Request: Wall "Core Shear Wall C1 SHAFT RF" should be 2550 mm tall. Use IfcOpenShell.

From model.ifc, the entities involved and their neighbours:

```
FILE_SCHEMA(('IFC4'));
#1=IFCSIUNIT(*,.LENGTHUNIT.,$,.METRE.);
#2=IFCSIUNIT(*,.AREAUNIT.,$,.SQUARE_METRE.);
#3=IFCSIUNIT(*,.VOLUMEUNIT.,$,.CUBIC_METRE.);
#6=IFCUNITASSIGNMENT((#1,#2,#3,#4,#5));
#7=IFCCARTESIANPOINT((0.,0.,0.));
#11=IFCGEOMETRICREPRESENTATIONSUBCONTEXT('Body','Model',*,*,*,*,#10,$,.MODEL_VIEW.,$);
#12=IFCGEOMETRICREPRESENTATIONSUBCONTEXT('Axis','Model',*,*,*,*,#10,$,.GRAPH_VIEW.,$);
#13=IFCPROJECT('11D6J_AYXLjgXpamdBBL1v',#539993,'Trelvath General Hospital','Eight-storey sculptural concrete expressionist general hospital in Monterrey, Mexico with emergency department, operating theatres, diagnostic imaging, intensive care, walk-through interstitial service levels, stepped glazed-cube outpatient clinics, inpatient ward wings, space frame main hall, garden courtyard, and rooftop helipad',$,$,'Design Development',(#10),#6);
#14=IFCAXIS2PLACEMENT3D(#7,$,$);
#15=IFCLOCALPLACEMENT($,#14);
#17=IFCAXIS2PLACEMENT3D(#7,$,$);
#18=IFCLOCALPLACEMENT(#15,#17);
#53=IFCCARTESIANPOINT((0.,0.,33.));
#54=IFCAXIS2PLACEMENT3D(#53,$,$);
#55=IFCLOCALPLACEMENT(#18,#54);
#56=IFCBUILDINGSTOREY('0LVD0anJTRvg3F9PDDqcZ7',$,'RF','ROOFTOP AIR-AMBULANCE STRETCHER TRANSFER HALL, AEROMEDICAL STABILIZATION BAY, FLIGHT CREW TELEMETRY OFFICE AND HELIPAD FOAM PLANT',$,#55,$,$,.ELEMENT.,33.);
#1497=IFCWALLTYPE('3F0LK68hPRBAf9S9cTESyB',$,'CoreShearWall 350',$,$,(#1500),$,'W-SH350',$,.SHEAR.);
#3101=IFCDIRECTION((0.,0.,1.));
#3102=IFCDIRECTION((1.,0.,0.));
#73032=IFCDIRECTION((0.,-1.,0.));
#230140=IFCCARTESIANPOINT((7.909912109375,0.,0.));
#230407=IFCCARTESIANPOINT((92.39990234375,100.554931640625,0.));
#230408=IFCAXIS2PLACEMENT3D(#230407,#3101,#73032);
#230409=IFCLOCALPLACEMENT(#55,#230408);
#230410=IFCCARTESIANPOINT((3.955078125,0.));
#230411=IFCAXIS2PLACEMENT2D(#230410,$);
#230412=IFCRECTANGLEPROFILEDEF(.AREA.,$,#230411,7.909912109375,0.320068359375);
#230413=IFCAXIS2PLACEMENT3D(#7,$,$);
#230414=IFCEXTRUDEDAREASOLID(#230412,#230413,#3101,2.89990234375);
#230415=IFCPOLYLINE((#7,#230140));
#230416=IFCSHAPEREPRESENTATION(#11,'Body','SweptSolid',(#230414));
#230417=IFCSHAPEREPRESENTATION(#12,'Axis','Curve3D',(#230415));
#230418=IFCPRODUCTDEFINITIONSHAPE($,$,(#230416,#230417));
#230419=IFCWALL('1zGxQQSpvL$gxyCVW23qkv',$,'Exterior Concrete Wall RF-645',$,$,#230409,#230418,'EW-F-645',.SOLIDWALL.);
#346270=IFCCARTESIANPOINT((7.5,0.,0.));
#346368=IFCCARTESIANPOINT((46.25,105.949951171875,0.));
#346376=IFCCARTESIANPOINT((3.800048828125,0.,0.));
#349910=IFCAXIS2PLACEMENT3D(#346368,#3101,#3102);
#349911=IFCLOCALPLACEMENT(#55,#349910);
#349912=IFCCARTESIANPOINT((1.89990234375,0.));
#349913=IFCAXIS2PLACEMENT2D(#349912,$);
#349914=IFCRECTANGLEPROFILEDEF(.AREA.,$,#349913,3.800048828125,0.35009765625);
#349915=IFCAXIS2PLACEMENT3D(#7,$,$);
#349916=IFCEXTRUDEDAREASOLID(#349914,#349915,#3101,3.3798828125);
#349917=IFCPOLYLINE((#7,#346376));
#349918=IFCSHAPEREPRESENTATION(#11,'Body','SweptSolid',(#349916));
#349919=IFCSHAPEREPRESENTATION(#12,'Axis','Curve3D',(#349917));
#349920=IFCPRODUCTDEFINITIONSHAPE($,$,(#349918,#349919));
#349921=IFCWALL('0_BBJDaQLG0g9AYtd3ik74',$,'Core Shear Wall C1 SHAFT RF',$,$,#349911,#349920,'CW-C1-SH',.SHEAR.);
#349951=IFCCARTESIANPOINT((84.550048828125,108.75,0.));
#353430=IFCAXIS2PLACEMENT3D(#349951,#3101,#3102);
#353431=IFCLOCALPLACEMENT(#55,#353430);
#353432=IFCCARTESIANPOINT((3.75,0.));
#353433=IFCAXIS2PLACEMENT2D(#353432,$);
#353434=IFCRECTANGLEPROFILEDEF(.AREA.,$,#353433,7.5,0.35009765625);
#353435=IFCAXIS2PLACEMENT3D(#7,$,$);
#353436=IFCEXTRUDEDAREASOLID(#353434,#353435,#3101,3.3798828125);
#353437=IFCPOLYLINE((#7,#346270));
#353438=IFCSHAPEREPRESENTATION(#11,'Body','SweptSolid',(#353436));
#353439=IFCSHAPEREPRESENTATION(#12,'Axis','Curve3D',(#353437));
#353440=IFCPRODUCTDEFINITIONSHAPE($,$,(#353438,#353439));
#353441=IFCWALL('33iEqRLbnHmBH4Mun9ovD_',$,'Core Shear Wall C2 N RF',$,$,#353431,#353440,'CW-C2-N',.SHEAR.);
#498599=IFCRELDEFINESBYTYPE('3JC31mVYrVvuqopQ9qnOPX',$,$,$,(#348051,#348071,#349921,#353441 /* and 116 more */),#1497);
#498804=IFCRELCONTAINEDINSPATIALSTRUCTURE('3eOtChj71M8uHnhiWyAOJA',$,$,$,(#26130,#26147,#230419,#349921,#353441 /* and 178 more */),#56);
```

```python
import ifcopenshell
import ifcopenshell.geom
import ifcopenshell.util.representation
import ifcopenshell.util.shape
import ifcopenshell.util.unit

model = ifcopenshell.open("model.ifc")
unit_scale = ifcopenshell.util.unit.calculate_unit_scale(model)
settings = ifcopenshell.geom.settings()


def volume(element):
    """Net volume in cubic metres, openings subtracted."""
    shape = ifcopenshell.geom.create_shape(settings, element)
    return ifcopenshell.util.shape.get_volume(shape.geometry)


wall = model.by_guid("0_BBJDaQLG0g9AYtd3ik74")
before = volume(wall)

body = ifcopenshell.util.representation.get_representation(wall, "Model", "Body")
solid = body.Items[0]
old_height = solid.Depth
solid.Depth = 2.55 / unit_scale
after = volume(wall)

print(f"height {old_height:g} -> {solid.Depth:g}, volume {before:.3f} -> {after:.3f} m3")

model.write("model_edited.ifc")
```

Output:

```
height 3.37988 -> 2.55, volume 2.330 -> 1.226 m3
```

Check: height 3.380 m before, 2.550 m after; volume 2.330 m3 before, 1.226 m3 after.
